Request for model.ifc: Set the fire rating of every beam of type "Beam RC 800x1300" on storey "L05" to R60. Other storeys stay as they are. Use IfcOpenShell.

First a look at what the model holds.

```python
import ifcopenshell
import ifcopenshell.util.element

model = ifcopenshell.open("model.ifc")
print(model.schema)
storey = next(s for s in model.by_type("IfcBuildingStorey") if s.Name == "L05")
beams = [e for e in ifcopenshell.util.element.get_decomposition(storey) if e.is_a("IfcBeam")]
seen = {}
for e in beams:
    element_type = ifcopenshell.util.element.get_type(e)
    key = (element_type.Name if element_type != e and element_type else None, ifcopenshell.util.element.get_pset(e, "Pset_BeamCommon", "FireRating"))
    seen[key] = seen.get(key, 0) + 1
for (name, value), count in sorted(seen.items(), key=str):
    print(count, "x", name, "|", value)
```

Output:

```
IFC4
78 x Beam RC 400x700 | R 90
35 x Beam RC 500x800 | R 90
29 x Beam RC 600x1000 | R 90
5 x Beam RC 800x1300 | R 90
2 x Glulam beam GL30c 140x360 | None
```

```python
import ifcopenshell
import ifcopenshell.api.pset
import ifcopenshell.util.element

model = ifcopenshell.open("model.ifc")

storey = next(s for s in model.by_type("IfcBuildingStorey") if s.Name == "L05")
beams = [e for e in ifcopenshell.util.element.get_decomposition(storey) if e.is_a("IfcBeam")]

count = 0
for e in beams:
    element_type = ifcopenshell.util.element.get_type(e)
    if element_type in (None, e) or element_type.Name != "Beam RC 800x1300":
        continue
    # add_pset returns the element's existing set when there is one.
    pset = ifcopenshell.api.pset.add_pset(model, product=e, name="Pset_BeamCommon")
    ifcopenshell.api.pset.edit_pset(model, pset=pset, properties={"FireRating": "R60"})
    count += 1

print(count, "beams updated")

model.write("model_v2.ifc")
```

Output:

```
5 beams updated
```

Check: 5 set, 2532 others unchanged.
